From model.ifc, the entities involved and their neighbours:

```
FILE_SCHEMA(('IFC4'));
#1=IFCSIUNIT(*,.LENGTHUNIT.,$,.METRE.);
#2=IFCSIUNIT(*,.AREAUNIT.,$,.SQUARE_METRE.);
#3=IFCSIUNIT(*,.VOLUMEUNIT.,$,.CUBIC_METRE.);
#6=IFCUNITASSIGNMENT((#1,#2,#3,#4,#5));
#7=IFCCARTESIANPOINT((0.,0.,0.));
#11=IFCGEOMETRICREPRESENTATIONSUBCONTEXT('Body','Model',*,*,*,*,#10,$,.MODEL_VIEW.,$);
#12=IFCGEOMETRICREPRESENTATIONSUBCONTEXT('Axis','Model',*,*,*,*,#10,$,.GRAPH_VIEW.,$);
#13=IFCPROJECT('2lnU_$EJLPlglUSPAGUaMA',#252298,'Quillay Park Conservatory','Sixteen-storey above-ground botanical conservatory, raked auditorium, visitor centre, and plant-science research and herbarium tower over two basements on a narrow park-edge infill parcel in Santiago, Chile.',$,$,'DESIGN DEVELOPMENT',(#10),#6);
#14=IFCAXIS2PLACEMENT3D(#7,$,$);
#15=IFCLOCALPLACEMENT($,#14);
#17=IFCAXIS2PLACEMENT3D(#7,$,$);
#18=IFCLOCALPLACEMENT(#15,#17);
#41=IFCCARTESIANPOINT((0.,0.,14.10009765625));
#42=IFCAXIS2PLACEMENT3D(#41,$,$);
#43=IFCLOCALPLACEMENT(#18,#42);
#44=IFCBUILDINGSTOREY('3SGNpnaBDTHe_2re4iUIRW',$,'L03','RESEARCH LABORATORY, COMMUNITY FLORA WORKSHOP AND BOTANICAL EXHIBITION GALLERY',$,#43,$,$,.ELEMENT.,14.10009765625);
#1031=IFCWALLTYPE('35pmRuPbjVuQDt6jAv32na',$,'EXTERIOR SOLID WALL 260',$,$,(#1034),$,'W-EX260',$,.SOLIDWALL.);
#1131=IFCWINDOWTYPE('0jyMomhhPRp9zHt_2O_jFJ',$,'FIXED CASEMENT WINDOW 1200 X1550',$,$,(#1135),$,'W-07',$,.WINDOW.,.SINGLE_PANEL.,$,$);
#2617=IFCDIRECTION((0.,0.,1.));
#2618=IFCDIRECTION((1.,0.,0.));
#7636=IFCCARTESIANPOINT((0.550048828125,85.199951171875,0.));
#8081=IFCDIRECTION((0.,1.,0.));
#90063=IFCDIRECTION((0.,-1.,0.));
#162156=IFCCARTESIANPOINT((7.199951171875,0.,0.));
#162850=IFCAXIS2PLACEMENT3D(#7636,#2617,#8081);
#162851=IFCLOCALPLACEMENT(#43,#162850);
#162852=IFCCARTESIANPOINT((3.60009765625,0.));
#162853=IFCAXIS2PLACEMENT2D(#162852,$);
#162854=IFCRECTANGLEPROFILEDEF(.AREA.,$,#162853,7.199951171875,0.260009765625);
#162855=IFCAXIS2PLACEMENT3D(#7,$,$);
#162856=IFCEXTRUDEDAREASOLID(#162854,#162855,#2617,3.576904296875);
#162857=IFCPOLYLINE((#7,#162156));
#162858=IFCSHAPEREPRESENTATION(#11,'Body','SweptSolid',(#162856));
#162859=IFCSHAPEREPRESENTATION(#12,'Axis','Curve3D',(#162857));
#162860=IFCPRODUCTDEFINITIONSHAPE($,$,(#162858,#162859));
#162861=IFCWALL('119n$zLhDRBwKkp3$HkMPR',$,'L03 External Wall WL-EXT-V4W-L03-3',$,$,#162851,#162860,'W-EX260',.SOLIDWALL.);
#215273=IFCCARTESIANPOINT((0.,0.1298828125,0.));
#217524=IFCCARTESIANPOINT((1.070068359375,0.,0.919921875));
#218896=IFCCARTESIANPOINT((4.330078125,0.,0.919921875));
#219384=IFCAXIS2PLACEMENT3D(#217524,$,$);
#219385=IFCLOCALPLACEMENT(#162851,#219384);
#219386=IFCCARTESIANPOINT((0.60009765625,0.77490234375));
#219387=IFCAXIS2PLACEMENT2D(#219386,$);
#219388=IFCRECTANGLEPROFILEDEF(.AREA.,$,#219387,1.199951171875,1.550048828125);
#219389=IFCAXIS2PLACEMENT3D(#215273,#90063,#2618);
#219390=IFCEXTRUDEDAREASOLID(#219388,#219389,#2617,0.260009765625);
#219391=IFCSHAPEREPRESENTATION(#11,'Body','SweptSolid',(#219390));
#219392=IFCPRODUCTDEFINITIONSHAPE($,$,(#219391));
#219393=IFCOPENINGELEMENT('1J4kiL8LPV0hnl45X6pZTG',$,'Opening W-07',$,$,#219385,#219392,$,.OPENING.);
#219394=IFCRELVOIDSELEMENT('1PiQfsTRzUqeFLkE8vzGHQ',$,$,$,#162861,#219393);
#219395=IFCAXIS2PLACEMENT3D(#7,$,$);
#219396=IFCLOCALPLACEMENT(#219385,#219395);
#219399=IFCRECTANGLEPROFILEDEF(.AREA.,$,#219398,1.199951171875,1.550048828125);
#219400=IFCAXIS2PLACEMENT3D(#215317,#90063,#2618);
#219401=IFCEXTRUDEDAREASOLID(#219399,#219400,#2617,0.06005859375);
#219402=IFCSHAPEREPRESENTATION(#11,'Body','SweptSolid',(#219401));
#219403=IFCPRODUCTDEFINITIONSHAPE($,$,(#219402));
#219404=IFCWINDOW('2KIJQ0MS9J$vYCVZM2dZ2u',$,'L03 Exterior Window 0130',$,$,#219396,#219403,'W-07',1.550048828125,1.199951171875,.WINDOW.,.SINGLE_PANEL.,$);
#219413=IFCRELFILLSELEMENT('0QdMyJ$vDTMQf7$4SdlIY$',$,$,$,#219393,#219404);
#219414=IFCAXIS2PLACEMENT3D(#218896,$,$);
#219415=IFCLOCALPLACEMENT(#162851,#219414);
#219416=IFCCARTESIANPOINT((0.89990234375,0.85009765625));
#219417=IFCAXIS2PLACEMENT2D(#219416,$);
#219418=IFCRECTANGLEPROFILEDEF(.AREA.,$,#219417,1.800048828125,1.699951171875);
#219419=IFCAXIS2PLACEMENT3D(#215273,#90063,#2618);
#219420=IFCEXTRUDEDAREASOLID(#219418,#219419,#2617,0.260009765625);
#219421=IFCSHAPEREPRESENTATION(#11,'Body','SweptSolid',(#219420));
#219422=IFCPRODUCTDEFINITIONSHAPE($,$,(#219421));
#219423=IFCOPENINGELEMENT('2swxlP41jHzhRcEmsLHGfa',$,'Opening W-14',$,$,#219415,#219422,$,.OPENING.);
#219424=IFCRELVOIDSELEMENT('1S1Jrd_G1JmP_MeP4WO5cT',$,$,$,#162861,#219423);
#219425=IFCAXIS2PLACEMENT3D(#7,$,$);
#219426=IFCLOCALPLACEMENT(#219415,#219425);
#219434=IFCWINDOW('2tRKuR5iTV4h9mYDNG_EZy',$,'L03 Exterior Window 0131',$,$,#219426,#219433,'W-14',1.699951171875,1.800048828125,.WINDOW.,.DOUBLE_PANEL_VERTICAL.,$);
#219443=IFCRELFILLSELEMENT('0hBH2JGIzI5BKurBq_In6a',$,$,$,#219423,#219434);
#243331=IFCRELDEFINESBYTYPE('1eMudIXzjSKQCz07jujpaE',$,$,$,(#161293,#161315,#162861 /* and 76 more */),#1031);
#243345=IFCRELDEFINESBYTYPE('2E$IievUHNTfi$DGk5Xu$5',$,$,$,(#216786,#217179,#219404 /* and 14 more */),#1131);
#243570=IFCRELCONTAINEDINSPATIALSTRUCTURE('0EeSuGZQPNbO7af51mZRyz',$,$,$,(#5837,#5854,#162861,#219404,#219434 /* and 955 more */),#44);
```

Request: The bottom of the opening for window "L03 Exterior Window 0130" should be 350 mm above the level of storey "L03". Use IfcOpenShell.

```python
import numpy as np
import ifcopenshell
import ifcopenshell.api.geometry
import ifcopenshell.geom
import ifcopenshell.util.element
import ifcopenshell.util.placement
import ifcopenshell.util.shape
import ifcopenshell.util.unit

model = ifcopenshell.open("model.ifc")
unit_scale = ifcopenshell.util.unit.calculate_unit_scale(model)

window = model.by_id(219404)
opening = window.FillsVoids[0].RelatingOpeningElement
storey = ifcopenshell.util.element.get_container(window, ifc_class="IfcBuildingStorey")
level = ifcopenshell.util.placement.get_local_placement(storey.ObjectPlacement)[2, 3]

# The opening's origin need not be at the sill, so measure its lowest point.
shape = ifcopenshell.geom.create_shape(ifcopenshell.geom.settings(), opening)
bottom = ifcopenshell.util.shape.get_shape_bottom_elevation(shape, shape.geometry) / unit_scale
dz = level + 0.35 - bottom

shift = np.array([0.0, 0.0, dz])
# The window is placed relative to its opening, so it follows when the opening moves.
matrix = ifcopenshell.util.placement.get_local_placement(opening.ObjectPlacement)
matrix[:3, 3] += shift
ifcopenshell.api.geometry.edit_object_placement(
    model, product=opening, matrix=matrix, is_si=False, should_transform_children=True
)

print(f"moved by {dz * unit_scale:+.3f} m")

model.write("model-out.ifc")
```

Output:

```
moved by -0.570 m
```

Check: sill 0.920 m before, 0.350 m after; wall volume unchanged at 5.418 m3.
